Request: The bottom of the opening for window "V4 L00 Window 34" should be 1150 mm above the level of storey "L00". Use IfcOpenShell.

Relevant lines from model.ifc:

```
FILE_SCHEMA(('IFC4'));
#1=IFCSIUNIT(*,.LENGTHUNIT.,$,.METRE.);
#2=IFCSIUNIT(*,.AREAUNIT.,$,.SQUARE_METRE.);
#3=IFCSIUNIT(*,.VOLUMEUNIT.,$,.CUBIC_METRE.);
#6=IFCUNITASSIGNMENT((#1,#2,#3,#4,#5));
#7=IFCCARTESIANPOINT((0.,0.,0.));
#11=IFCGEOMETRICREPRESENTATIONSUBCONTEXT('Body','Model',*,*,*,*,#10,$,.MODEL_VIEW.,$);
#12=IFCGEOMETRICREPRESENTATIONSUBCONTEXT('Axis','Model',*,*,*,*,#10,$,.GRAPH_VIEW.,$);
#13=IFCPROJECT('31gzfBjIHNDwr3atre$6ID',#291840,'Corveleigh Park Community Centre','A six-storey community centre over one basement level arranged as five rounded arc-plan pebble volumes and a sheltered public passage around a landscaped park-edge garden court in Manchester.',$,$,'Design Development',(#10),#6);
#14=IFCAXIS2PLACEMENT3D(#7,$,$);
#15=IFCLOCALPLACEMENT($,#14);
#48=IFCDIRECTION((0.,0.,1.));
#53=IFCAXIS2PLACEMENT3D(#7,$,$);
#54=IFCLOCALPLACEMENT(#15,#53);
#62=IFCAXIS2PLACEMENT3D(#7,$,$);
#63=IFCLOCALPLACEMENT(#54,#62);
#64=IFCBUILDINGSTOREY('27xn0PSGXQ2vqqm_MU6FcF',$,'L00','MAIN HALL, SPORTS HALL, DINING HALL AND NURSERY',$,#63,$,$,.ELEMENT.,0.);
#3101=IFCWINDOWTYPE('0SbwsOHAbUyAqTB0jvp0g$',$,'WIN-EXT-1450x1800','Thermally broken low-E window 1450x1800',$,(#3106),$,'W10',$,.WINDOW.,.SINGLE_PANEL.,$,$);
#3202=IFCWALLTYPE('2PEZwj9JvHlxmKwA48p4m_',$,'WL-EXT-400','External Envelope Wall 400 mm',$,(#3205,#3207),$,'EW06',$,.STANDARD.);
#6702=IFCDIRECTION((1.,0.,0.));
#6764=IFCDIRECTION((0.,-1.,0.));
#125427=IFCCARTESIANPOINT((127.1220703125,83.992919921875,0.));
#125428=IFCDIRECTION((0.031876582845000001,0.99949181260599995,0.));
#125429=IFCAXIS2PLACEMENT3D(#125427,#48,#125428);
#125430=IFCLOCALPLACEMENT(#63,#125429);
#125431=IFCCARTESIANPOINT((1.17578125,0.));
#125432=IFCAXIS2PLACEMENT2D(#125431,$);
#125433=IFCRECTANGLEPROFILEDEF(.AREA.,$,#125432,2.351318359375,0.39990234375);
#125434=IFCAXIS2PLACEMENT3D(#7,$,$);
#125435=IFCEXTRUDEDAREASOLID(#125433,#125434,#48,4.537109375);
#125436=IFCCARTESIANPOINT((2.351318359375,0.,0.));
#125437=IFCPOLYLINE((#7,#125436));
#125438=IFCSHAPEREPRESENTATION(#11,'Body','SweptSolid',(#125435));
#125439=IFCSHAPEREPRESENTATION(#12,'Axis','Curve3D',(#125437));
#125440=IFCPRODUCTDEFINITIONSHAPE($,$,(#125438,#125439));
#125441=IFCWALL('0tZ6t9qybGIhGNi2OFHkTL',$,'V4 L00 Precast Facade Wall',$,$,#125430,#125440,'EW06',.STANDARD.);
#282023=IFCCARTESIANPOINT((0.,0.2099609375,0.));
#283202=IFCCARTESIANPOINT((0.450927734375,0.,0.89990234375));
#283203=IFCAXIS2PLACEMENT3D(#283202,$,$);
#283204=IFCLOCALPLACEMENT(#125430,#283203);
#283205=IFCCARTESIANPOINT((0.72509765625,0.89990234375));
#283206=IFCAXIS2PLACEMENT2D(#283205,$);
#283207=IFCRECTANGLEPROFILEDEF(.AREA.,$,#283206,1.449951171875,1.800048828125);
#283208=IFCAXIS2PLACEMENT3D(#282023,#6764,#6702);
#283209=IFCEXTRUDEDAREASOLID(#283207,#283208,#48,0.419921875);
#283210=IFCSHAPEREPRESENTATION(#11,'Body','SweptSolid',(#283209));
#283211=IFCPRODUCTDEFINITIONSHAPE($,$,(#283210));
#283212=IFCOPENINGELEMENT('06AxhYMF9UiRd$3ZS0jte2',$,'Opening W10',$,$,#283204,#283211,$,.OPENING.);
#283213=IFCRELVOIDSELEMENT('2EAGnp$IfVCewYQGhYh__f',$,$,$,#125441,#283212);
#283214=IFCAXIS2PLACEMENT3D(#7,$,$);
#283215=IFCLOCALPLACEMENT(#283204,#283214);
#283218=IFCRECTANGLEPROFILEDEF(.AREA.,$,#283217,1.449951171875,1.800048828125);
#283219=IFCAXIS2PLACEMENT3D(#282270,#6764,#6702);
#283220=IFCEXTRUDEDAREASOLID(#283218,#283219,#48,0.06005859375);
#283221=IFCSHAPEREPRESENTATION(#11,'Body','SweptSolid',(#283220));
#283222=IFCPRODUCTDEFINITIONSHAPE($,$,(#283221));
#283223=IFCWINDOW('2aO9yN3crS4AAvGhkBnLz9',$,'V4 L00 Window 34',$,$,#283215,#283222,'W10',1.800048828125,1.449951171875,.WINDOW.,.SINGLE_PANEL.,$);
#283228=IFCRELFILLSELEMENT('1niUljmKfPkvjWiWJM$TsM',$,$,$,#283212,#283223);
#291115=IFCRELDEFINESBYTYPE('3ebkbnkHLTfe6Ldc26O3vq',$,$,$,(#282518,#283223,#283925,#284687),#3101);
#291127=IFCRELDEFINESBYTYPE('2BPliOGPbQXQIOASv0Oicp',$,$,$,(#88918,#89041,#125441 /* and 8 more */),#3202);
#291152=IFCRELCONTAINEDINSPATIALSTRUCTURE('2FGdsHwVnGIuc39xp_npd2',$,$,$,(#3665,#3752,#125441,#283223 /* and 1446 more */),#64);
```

```python
import numpy as np
import ifcopenshell
import ifcopenshell.api.geometry
import ifcopenshell.geom
import ifcopenshell.util.element
import ifcopenshell.util.placement
import ifcopenshell.util.shape
import ifcopenshell.util.unit

model = ifcopenshell.open("model.ifc")
unit_scale = ifcopenshell.util.unit.calculate_unit_scale(model)

window = model.by_guid("2aO9yN3crS4AAvGhkBnLz9")
opening = window.FillsVoids[0].RelatingOpeningElement
storey = ifcopenshell.util.element.get_container(window, ifc_class="IfcBuildingStorey")
level = ifcopenshell.util.placement.get_local_placement(storey.ObjectPlacement)[2, 3]

# The opening's origin need not be at the sill, so measure its lowest point.
shape = ifcopenshell.geom.create_shape(ifcopenshell.geom.settings(), opening)
bottom = ifcopenshell.util.shape.get_shape_bottom_elevation(shape, shape.geometry) / unit_scale
dz = level + 1.15 - bottom

shift = np.array([0.0, 0.0, dz])
# The window is placed relative to its opening, so it follows when the opening moves.
matrix = ifcopenshell.util.placement.get_local_placement(opening.ObjectPlacement)
matrix[:3, 3] += shift
ifcopenshell.api.geometry.edit_object_placement(
    model, product=opening, matrix=matrix, is_si=False, should_transform_children=True
)

print(f"moved by {dz * unit_scale:+.3f} m")

model.write("model_updated.ifc")
```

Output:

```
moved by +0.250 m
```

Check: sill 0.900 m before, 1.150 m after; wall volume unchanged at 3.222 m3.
